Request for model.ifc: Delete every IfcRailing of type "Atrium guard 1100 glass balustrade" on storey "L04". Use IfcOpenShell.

First a look at what the model holds.

```python
import ifcopenshell
import ifcopenshell.util.element

model = ifcopenshell.open("model.ifc")
print(model.schema)
storey = next(s for s in model.by_type("IfcBuildingStorey") if s.Name == "L04")
railings = [e for e in ifcopenshell.util.element.get_decomposition(storey) if e.is_a("IfcRailing")]
seen = {}
for e in railings:
    element_type = ifcopenshell.util.element.get_type(e)
    name = element_type.Name if element_type not in (None, e) else None
    seen[name] = seen.get(name, 0) + 1
for name, count in sorted(seen.items(), key=str):
    print(count, "x", name)
```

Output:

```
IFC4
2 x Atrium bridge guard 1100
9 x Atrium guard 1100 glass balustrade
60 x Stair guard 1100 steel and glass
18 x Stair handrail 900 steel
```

```python
import ifcopenshell
import ifcopenshell.api.root
import ifcopenshell.util.element

model = ifcopenshell.open("model.ifc")

storey = next(s for s in model.by_type("IfcBuildingStorey") if s.Name == "L04")
railings = [e for e in ifcopenshell.util.element.get_decomposition(storey) if e.is_a("IfcRailing")]
targets = [e for e in railings if (t := ifcopenshell.util.element.get_type(e)) not in (None, e) and t.Name == "Atrium guard 1100 glass balustrade"]

for e in targets:
    ifcopenshell.api.root.remove_product(model, product=e)
print(len(targets), "removed")

model.write("model_rev.ifc")
```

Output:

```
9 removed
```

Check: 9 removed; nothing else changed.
